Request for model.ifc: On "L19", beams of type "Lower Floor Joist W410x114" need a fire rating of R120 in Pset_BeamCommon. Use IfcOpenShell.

First a look at what the model holds.

```python
import ifcopenshell
import ifcopenshell.util.element

model = ifcopenshell.open("model.ifc")
print(model.schema)
storey = next(s for s in model.by_type("IfcBuildingStorey") if s.Name == "L19")
beams = [e for e in ifcopenshell.util.element.get_decomposition(storey) if e.is_a("IfcBeam")]
seen = {}
for e in beams:
    element_type = ifcopenshell.util.element.get_type(e)
    key = (element_type.Name if element_type != e and element_type else None, ifcopenshell.util.element.get_pset(e, "Pset_BeamCommon", "FireRating"))
    seen[key] = seen.get(key, 0) + 1
for (name, value), count in sorted(seen.items(), key=str):
    print(count, "x", name, "|", value)
```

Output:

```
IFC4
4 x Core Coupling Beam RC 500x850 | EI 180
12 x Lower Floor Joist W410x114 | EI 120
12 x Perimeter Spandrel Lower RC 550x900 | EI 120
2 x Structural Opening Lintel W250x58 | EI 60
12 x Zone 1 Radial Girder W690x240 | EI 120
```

```python
import ifcopenshell
import ifcopenshell.api.pset
import ifcopenshell.util.element

model = ifcopenshell.open("model.ifc")

storey = next(s for s in model.by_type("IfcBuildingStorey") if s.Name == "L19")
beams = [e for e in ifcopenshell.util.element.get_decomposition(storey) if e.is_a("IfcBeam")]

count = 0
for e in beams:
    element_type = ifcopenshell.util.element.get_type(e)
    if element_type in (None, e) or element_type.Name != "Lower Floor Joist W410x114":
        continue
    found = ifcopenshell.util.element.get_pset(e, "Pset_BeamCommon", should_inherit=False)
    if found:
        pset = model.by_id(found["id"])
        if len(ifcopenshell.util.element.get_elements_by_pset(pset)) > 1:
            pset = ifcopenshell.api.pset.unshare_pset(model, products=[e], pset=pset)[0]
    else:
        pset = ifcopenshell.api.pset.add_pset(model, product=e, name="Pset_BeamCommon")
    ifcopenshell.api.pset.edit_pset(model, pset=pset, properties={"FireRating": "R120"})
    count += 1

print(count, "beams updated")

model.write("model_updated.ifc")
```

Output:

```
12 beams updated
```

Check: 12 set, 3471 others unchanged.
